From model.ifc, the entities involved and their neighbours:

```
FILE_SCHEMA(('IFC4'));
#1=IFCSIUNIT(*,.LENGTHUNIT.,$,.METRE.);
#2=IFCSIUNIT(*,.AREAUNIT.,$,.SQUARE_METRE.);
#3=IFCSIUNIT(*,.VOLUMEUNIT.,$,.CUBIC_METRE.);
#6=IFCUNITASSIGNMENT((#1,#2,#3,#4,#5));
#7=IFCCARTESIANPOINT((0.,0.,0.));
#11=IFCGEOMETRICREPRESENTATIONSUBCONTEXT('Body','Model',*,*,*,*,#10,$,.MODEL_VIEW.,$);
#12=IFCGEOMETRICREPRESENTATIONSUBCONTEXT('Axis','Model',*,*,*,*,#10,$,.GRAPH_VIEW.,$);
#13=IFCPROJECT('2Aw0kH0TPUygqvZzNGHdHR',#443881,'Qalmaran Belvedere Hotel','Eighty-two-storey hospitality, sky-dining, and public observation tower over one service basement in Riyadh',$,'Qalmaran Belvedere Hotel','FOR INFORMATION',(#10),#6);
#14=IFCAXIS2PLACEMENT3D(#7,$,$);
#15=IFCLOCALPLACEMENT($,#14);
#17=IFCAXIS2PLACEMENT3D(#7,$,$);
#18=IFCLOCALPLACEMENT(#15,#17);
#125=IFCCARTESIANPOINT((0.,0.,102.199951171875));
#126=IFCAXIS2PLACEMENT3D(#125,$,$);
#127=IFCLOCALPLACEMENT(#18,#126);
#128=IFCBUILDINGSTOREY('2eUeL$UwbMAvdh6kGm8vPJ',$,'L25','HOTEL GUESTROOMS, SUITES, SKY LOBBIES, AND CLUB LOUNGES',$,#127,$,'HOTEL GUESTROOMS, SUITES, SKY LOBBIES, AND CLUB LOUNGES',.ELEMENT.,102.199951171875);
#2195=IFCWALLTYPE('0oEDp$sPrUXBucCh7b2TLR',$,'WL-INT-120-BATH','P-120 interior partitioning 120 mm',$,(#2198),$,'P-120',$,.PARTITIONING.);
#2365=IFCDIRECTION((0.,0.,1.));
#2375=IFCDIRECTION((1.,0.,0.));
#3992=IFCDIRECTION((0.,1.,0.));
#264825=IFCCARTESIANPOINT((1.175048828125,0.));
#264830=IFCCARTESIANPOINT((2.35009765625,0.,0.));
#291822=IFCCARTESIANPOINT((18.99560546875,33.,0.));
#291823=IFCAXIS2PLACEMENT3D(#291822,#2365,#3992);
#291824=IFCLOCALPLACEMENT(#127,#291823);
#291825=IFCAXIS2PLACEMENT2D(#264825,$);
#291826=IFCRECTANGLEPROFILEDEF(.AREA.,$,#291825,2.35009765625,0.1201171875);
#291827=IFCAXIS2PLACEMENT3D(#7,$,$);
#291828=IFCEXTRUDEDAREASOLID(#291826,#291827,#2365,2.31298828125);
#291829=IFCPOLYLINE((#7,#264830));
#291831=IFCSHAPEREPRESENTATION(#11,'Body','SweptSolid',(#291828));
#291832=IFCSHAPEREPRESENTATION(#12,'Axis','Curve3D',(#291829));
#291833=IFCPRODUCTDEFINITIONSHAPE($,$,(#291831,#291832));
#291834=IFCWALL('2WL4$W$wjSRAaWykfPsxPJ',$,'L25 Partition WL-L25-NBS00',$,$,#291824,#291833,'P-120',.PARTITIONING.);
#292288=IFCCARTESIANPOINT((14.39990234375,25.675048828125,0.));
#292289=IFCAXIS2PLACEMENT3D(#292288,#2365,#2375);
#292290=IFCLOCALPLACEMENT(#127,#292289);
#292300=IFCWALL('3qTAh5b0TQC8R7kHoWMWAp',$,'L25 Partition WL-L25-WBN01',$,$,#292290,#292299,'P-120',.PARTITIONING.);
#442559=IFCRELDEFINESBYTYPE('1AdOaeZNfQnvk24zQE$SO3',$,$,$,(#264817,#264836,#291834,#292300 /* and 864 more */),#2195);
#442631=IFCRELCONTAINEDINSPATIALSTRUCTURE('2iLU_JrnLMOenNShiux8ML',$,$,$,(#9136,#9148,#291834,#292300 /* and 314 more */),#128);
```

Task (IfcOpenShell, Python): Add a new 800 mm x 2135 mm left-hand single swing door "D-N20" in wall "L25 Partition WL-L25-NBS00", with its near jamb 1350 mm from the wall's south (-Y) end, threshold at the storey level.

```python
import numpy as np
import ifcopenshell
import ifcopenshell.api.feature
import ifcopenshell.api.geometry
import ifcopenshell.api.root
import ifcopenshell.api.spatial
import ifcopenshell.geom
import ifcopenshell.util.element
import ifcopenshell.util.placement
import ifcopenshell.util.representation
import ifcopenshell.util.shape
import ifcopenshell.util.unit

model = ifcopenshell.open("model.ifc")
unit_scale = ifcopenshell.util.unit.calculate_unit_scale(model)
settings = ifcopenshell.geom.settings()


def volume(element):
    """Net volume in cubic metres, openings subtracted."""
    shape = ifcopenshell.geom.create_shape(settings, element)
    return ifcopenshell.util.shape.get_volume(shape.geometry)


wall = model.by_guid("2WL4$W$wjSRAaWykfPsxPJ")
storey = ifcopenshell.util.element.get_container(wall, ifc_class="IfcBuildingStorey")
context = ifcopenshell.util.representation.get_context(model, "Model", "Body", "MODEL_VIEW")
before = volume(wall)

width, height, from_end, sill = 0.8, 2.135, 1.35, 0.0  # metres

# The wall runs along its own X axis, and the end named is its -X end.
wall_shape = ifcopenshell.geom.create_shape(settings, wall)
x, y, z = ifcopenshell.util.shape.get_vertices(wall_shape.geometry).T
start = x.min() + from_end
face, thickness = float(y.min()), float(y.max() - y.min())
wall_matrix = ifcopenshell.util.placement.get_local_placement(wall.ObjectPlacement)
level = ifcopenshell.util.placement.get_local_placement(storey.ObjectPlacement)[2, 3]


def in_wall(x, y):
    """Placement at x, y metres in the wall's axes, at sill height."""
    matrix = wall_matrix.copy()
    matrix[:, 3] = wall_matrix @ np.array([x / unit_scale, y / unit_scale, 0.0, 1.0])
    matrix[2, 3] = level + sill / unit_scale
    return matrix


# Opening: a box that overshoots both wall faces by 50 mm.
opening = ifcopenshell.api.root.create_entity(model, ifc_class="IfcOpeningElement", predefined_type="OPENING")
box = ifcopenshell.api.geometry.add_wall_representation(
    model, context=context, length=width, height=height, thickness=thickness + 0.1
)
ifcopenshell.api.geometry.assign_representation(model, product=opening, representation=box)
ifcopenshell.api.geometry.edit_object_placement(model, product=opening, matrix=in_wall(start, face - 0.05), is_si=False)
ifcopenshell.api.feature.add_feature(model, feature=opening, element=wall)

door = ifcopenshell.api.root.create_entity(model, ifc_class="IfcDoor", name="D-N20", predefined_type="DOOR")
door.OverallWidth, door.OverallHeight = width / unit_scale, height / unit_scale
door.OperationType = "SINGLE_SWING_LEFT"
body = ifcopenshell.api.geometry.add_door_representation(
    model,
    context=context,
    overall_width=door.OverallWidth,
    overall_height=door.OverallHeight,
    operation_type="SINGLE_SWING_LEFT",
    lining_properties={"LiningDepth": thickness / unit_scale, "ThresholdDepth": thickness / unit_scale},
)
ifcopenshell.api.geometry.assign_representation(model, product=door, representation=body)
ifcopenshell.api.spatial.assign_container(model, products=[door], relating_structure=storey)
ifcopenshell.api.feature.add_filling(model, opening=opening, element=door)

# The lining spans the wall, so the door starts at the wall face.
ifcopenshell.api.geometry.edit_object_placement(model, product=door, matrix=in_wall(start, face), is_si=False)

after = volume(wall)

print(f"wall volume {before:.3f} -> {after:.3f} m3")

model.write("model-out.ifc")
```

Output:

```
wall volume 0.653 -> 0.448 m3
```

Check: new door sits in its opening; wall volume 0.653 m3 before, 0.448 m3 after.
